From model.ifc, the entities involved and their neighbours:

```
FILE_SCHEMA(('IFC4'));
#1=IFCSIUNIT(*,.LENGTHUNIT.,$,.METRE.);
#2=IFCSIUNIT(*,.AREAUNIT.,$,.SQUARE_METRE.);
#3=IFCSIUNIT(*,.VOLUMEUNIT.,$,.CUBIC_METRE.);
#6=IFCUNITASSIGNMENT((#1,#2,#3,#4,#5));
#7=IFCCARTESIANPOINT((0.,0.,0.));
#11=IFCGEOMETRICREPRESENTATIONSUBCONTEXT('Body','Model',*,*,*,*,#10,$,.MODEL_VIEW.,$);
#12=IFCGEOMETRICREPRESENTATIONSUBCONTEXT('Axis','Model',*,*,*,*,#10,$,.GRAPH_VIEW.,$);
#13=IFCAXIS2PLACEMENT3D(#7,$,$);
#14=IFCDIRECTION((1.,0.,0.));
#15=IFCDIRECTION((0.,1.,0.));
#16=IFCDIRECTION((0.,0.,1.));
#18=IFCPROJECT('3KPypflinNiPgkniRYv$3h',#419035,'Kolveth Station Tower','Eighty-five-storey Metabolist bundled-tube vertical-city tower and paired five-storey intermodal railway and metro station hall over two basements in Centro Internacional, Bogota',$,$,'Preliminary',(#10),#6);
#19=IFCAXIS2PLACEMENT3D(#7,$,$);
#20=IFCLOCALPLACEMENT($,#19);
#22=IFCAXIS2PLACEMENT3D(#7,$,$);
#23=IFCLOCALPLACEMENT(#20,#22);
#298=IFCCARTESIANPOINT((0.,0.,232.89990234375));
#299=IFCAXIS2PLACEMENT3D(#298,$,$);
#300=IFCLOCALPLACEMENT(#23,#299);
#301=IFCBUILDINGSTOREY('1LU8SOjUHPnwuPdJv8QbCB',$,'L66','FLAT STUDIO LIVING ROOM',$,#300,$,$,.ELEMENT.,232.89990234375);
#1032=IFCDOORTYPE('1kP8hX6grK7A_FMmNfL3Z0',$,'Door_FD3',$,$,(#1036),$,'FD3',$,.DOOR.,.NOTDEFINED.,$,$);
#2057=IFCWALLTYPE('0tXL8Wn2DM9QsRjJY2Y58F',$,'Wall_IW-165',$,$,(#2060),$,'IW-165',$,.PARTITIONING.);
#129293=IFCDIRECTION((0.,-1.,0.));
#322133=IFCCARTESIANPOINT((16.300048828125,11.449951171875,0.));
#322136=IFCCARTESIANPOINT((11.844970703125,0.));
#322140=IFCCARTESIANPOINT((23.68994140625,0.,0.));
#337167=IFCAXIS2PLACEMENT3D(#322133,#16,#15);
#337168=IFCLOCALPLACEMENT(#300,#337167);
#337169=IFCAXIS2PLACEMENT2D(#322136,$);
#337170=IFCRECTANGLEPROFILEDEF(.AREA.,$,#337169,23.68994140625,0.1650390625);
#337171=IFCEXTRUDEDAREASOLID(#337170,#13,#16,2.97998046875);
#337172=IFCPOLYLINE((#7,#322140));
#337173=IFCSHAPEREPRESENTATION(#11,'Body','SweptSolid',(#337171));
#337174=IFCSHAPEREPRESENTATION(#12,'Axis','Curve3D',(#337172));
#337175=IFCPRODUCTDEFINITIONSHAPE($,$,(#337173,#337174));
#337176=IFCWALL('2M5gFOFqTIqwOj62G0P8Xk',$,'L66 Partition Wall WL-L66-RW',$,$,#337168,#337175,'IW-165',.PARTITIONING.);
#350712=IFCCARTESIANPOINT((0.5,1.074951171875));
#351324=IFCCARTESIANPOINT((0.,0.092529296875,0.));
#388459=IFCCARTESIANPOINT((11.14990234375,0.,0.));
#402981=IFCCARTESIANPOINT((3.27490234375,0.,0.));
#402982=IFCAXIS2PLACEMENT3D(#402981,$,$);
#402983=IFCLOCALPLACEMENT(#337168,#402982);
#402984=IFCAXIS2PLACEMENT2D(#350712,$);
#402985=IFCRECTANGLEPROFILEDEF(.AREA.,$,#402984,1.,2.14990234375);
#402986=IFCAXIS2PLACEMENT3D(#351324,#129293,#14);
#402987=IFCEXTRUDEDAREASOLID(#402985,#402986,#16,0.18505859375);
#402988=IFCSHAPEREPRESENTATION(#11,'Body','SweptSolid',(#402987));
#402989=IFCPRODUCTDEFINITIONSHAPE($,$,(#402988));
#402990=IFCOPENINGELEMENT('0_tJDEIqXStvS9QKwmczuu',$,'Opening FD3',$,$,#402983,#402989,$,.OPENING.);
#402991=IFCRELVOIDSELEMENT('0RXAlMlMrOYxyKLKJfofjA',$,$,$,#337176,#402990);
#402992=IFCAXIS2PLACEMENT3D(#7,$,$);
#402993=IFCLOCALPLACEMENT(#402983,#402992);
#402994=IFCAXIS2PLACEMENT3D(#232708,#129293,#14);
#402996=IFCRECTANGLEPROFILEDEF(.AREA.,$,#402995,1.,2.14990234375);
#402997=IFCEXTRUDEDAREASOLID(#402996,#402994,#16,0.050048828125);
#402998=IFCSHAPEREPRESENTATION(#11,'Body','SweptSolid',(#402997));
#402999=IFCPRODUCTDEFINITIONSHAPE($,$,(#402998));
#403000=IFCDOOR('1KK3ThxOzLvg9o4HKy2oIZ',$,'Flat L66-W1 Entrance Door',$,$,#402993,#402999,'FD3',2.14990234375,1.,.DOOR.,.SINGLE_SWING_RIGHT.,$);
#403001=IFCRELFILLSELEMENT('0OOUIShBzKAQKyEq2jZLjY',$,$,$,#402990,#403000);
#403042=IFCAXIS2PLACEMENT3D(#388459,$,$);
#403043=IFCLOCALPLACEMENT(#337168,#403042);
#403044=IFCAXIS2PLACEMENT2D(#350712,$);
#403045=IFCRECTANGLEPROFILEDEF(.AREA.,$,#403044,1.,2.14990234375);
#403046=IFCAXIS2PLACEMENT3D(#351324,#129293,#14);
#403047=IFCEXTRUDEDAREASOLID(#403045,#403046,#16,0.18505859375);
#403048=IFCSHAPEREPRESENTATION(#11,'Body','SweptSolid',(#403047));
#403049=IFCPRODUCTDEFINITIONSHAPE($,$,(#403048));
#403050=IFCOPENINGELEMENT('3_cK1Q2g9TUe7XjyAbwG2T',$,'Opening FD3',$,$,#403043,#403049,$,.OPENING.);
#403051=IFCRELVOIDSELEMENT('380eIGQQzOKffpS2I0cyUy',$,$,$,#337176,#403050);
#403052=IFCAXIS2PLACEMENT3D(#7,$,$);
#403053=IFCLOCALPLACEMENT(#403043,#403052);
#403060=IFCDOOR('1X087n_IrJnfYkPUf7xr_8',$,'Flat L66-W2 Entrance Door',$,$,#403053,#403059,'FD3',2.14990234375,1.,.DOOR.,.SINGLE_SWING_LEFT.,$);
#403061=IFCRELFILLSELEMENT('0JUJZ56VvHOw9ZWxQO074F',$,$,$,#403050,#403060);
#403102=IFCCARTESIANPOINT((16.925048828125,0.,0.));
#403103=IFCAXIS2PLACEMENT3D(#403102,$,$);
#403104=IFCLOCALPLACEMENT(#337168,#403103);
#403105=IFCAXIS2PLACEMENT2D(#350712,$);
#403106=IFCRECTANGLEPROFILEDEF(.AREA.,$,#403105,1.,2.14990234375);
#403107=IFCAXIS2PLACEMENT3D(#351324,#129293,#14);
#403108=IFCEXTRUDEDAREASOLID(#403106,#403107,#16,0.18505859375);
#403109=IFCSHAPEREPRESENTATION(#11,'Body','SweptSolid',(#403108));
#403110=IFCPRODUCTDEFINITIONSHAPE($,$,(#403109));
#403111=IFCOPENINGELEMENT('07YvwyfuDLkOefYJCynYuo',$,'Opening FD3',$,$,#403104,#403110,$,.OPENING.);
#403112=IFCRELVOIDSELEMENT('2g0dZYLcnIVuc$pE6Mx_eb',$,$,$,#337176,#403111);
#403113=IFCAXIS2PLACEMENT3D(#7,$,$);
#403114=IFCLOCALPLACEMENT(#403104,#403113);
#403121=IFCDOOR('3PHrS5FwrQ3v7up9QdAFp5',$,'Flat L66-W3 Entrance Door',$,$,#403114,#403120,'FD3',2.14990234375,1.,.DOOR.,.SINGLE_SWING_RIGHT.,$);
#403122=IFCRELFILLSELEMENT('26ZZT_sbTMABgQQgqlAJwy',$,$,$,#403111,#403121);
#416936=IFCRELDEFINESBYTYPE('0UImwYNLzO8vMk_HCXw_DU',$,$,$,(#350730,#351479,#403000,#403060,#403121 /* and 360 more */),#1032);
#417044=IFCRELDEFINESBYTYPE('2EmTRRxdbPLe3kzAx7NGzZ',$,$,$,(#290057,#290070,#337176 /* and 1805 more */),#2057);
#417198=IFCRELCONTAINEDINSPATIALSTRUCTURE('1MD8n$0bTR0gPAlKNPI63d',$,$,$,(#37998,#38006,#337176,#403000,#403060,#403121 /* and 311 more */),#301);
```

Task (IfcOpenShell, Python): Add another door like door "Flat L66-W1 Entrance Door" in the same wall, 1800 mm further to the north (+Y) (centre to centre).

```python
import ifcopenshell
import ifcopenshell.api.feature
import ifcopenshell.api.geometry
import ifcopenshell.api.root
import ifcopenshell.geom
import ifcopenshell.util.element
import ifcopenshell.util.placement
import ifcopenshell.util.shape

model = ifcopenshell.open("model.ifc")
settings = ifcopenshell.geom.settings()


def volume(element):
    """Net volume in cubic metres, openings subtracted."""
    shape = ifcopenshell.geom.create_shape(settings, element)
    return ifcopenshell.util.shape.get_volume(shape.geometry)


door = model.by_id(403000)
opening = door.FillsVoids[0].RelatingOpeningElement
wall = opening.VoidsElements[0].RelatingBuildingElement
before = volume(wall)
shift = ifcopenshell.util.placement.get_local_placement(wall.ObjectPlacement)[:3, 0] * 1.8

# copy_class copies the void relationship, type, container and properties, but no geometry.
new_opening = ifcopenshell.api.root.copy_class(model, product=opening)
new_opening.Representation = ifcopenshell.util.element.copy_deep(
    model, opening.Representation, exclude=["IfcGeometricRepresentationContext", "IfcRepresentationMap"]
)
new_door = ifcopenshell.api.root.copy_class(model, product=door)
new_door.Representation = ifcopenshell.util.element.copy_deep(
    model, door.Representation, exclude=["IfcGeometricRepresentationContext", "IfcRepresentationMap"]
)
new_door.Tag = None
ifcopenshell.api.feature.add_filling(model, opening=new_opening, element=new_door)

for old, new in ((opening, new_opening), (door, new_door)):
    matrix = ifcopenshell.util.placement.get_local_placement(old.ObjectPlacement)
    matrix[:3, 3] += shift
    ifcopenshell.api.geometry.edit_object_placement(model, product=new, matrix=matrix, is_si=False)

after = volume(wall)

print(f"wall volume {before:.3f} -> {after:.3f} m3")

model.write("model-out.ifc")
```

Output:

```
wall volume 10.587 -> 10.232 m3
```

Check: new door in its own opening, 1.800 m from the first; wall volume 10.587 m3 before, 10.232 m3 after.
